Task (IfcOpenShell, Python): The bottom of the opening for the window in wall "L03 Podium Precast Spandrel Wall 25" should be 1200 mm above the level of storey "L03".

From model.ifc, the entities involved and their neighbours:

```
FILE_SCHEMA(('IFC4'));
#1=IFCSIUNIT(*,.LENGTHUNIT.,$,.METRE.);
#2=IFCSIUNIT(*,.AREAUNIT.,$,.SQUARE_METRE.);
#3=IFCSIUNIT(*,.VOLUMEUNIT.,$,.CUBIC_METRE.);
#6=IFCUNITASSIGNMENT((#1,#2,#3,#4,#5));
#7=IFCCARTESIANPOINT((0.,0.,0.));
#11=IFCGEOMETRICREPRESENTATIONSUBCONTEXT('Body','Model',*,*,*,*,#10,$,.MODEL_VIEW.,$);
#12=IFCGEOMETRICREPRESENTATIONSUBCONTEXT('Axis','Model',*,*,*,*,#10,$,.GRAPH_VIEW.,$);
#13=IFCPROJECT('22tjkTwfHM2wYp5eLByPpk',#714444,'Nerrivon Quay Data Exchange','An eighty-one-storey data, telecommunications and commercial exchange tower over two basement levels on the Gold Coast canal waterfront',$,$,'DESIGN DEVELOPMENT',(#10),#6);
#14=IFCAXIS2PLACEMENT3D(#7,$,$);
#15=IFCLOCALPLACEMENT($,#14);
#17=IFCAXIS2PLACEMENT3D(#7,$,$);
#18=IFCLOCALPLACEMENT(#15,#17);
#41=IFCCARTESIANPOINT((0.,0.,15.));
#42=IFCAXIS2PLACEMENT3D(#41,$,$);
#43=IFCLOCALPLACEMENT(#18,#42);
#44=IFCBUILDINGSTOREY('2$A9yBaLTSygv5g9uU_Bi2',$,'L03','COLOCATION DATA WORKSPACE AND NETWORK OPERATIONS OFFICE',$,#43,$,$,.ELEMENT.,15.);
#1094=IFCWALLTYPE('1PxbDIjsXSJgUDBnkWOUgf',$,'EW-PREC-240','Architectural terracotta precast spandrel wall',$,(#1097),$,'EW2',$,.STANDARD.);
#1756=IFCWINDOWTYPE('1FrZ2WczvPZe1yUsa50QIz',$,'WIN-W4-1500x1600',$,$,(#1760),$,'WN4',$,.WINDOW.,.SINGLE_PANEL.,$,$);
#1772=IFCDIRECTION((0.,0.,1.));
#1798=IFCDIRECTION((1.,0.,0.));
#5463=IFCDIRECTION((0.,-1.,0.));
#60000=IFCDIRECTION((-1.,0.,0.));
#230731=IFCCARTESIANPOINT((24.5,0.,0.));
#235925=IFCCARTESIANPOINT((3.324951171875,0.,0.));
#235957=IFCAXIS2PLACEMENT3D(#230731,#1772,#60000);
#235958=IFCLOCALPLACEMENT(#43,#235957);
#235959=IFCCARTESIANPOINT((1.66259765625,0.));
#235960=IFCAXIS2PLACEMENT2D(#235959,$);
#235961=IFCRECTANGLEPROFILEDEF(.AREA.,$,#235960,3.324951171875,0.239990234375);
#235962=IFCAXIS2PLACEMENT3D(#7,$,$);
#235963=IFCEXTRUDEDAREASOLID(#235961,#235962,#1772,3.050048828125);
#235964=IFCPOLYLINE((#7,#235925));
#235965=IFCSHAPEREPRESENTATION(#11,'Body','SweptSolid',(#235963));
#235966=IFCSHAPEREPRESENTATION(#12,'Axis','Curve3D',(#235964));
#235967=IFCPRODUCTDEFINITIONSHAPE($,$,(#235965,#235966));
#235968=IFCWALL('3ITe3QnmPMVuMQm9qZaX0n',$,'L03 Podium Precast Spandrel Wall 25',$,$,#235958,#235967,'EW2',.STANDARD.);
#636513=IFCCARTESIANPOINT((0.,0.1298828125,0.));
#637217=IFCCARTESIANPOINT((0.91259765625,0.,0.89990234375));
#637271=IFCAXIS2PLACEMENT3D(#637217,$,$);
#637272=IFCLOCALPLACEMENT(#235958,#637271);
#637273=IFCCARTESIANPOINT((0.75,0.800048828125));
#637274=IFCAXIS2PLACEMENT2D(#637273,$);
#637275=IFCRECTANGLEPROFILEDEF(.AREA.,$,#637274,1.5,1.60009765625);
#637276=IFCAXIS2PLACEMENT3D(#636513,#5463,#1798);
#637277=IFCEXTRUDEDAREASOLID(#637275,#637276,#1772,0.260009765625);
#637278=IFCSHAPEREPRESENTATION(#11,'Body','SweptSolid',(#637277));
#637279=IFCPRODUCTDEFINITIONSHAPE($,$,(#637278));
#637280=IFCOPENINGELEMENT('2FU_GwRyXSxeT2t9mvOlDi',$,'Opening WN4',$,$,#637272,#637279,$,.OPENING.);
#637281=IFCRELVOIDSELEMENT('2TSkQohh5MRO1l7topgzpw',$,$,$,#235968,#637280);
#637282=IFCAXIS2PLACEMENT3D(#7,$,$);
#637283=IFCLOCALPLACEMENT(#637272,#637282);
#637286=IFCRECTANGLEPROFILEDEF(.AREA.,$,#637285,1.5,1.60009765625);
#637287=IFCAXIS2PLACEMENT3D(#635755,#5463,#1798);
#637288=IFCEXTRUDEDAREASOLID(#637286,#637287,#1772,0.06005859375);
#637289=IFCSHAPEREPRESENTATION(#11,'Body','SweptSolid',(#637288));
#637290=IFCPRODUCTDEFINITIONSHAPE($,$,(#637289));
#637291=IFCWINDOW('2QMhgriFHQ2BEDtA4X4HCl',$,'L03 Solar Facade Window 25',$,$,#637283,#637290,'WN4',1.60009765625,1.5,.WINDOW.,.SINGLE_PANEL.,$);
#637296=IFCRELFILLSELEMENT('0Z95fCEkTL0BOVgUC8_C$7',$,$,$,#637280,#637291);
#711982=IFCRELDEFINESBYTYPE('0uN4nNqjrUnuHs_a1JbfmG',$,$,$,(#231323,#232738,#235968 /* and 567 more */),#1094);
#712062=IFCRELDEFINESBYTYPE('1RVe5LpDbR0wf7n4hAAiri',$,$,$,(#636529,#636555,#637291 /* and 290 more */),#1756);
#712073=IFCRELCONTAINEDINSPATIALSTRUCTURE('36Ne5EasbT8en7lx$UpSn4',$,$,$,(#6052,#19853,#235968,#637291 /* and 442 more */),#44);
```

```python
import numpy as np
import ifcopenshell
import ifcopenshell.api.geometry
import ifcopenshell.geom
import ifcopenshell.util.element
import ifcopenshell.util.placement
import ifcopenshell.util.shape
import ifcopenshell.util.unit

model = ifcopenshell.open("model.ifc")
unit_scale = ifcopenshell.util.unit.calculate_unit_scale(model)

window = model.by_guid("2QMhgriFHQ2BEDtA4X4HCl")
opening = window.FillsVoids[0].RelatingOpeningElement
storey = ifcopenshell.util.element.get_container(window, ifc_class="IfcBuildingStorey")
level = ifcopenshell.util.placement.get_local_placement(storey.ObjectPlacement)[2, 3]

# The opening's origin need not be at the sill, so measure its lowest point.
shape = ifcopenshell.geom.create_shape(ifcopenshell.geom.settings(), opening)
bottom = ifcopenshell.util.shape.get_shape_bottom_elevation(shape, shape.geometry) / unit_scale
dz = level + 1.2 - bottom

shift = np.array([0.0, 0.0, dz])
# The window is placed relative to its opening, so it follows when the opening moves.
matrix = ifcopenshell.util.placement.get_local_placement(opening.ObjectPlacement)
matrix[:3, 3] += shift
ifcopenshell.api.geometry.edit_object_placement(
    model, product=opening, matrix=matrix, is_si=False, should_transform_children=True
)

print(f"moved by {dz * unit_scale:+.3f} m")

model.write("model_v2.ifc")
```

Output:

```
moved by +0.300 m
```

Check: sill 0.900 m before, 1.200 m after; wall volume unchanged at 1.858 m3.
